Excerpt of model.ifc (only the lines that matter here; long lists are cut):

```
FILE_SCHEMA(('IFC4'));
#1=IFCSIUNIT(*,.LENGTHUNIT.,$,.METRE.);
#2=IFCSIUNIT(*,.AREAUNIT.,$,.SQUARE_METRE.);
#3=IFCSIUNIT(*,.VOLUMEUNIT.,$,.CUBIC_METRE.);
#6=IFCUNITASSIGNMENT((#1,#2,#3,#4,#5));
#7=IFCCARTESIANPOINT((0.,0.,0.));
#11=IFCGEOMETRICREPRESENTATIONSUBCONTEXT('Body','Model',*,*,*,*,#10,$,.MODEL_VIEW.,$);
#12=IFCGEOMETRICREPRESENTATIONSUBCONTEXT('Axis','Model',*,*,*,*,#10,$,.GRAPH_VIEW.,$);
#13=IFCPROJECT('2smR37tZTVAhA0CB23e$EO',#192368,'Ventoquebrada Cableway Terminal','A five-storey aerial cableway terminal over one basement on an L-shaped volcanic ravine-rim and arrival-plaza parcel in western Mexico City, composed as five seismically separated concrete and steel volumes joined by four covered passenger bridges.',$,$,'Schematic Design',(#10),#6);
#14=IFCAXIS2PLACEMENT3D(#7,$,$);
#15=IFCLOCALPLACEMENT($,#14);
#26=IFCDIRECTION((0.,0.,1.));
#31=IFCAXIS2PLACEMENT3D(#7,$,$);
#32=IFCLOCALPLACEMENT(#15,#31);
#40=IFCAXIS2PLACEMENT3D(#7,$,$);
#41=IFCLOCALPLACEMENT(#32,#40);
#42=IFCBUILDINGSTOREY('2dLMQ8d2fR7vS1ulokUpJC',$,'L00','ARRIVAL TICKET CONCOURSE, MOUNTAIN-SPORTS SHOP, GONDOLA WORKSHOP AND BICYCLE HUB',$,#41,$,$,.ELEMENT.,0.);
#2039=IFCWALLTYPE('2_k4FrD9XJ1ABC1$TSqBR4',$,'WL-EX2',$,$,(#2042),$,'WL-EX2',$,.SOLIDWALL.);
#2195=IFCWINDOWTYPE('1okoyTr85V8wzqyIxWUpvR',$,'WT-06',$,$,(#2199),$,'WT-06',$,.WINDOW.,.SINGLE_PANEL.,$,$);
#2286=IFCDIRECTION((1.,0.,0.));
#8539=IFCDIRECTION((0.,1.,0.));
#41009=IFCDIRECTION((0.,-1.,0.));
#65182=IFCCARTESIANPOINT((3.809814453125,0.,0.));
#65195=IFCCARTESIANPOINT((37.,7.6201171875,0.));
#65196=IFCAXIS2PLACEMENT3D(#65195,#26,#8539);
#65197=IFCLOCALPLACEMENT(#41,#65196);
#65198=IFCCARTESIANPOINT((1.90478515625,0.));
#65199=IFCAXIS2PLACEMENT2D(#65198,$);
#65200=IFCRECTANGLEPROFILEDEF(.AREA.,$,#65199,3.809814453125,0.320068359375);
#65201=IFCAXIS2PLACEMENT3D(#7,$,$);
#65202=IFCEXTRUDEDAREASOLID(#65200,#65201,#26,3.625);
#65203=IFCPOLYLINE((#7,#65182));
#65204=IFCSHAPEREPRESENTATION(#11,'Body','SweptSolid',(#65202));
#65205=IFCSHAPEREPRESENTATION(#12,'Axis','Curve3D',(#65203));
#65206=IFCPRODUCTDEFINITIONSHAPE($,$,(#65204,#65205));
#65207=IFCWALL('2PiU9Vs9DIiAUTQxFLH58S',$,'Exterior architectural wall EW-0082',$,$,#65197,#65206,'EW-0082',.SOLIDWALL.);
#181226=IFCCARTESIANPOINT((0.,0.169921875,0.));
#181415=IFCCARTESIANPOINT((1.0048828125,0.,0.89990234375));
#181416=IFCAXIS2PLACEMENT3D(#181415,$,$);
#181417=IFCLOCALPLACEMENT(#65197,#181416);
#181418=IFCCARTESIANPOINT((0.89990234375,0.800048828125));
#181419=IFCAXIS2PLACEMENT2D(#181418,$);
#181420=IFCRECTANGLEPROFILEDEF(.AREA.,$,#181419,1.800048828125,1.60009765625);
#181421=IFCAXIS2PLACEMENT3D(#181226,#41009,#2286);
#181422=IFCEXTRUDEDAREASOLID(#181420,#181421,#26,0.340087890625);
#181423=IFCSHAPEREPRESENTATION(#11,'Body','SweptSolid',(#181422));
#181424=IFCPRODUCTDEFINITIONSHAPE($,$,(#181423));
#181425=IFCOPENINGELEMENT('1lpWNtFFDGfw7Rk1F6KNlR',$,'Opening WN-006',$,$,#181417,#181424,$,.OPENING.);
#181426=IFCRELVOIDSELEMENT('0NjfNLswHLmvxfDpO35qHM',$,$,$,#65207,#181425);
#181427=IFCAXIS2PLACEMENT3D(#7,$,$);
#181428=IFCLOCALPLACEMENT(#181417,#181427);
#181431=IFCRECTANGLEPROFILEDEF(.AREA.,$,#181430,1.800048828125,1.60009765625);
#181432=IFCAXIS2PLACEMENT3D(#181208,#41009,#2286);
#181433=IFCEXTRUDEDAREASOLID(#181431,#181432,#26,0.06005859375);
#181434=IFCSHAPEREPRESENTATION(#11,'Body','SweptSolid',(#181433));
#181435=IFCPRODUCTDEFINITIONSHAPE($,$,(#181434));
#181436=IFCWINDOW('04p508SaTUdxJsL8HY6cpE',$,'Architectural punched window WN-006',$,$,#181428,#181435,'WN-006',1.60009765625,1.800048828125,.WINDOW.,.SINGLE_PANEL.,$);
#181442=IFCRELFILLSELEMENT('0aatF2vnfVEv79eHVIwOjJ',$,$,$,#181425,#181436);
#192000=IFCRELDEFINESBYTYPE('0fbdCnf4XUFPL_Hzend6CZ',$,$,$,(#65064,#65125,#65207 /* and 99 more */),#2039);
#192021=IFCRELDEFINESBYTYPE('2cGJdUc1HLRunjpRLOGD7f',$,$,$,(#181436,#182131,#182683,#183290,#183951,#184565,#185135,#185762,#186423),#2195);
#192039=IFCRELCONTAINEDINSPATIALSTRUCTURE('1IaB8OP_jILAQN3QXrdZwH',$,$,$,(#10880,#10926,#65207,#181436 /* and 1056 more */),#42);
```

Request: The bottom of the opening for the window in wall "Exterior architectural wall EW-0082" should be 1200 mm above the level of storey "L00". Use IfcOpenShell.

```python
import numpy as np
import ifcopenshell
import ifcopenshell.api.geometry
import ifcopenshell.geom
import ifcopenshell.util.element
import ifcopenshell.util.placement
import ifcopenshell.util.shape
import ifcopenshell.util.unit

model = ifcopenshell.open("model.ifc")
unit_scale = ifcopenshell.util.unit.calculate_unit_scale(model)

window = model.by_guid("04p508SaTUdxJsL8HY6cpE")
opening = window.FillsVoids[0].RelatingOpeningElement
storey = ifcopenshell.util.element.get_container(window, ifc_class="IfcBuildingStorey")
level = ifcopenshell.util.placement.get_local_placement(storey.ObjectPlacement)[2, 3]

# The opening's origin need not be at the sill, so measure its lowest point.
shape = ifcopenshell.geom.create_shape(ifcopenshell.geom.settings(), opening)
bottom = ifcopenshell.util.shape.get_shape_bottom_elevation(shape, shape.geometry) / unit_scale
dz = level + 1.2 / unit_scale - bottom

shift = np.array([0.0, 0.0, dz])
# The window is placed relative to its opening, so it follows when the opening moves.
matrix = ifcopenshell.util.placement.get_local_placement(opening.ObjectPlacement)
matrix[:3, 3] += shift
ifcopenshell.api.geometry.edit_object_placement(
    model, product=opening, matrix=matrix, is_si=False, should_transform_children=True
)

print(f"moved by {dz * unit_scale:+.3f} m")

model.write("model_updated.ifc")
```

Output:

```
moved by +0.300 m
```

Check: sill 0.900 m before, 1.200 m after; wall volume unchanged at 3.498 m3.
